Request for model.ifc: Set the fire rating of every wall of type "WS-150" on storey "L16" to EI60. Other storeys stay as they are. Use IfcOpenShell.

First a look at what the model holds.

```python
import ifcopenshell
import ifcopenshell.util.element

model = ifcopenshell.open("model.ifc")
print(model.schema)
storey = next(s for s in model.by_type("IfcBuildingStorey") if s.Name == "L16")
walls = [e for e in ifcopenshell.util.element.get_decomposition(storey) if e.is_a("IfcWall")]
seen = {}
for e in walls:
    element_type = ifcopenshell.util.element.get_type(e)
    key = (element_type.Name if element_type != e and element_type else None, ifcopenshell.util.element.get_pset(e, "Pset_WallCommon", "FireRating"))
    seen[key] = seen.get(key, 0) + 1
for (name, value), count in sorted(seen.items(), key=str):
    print(count, "x", name, "|", value)
```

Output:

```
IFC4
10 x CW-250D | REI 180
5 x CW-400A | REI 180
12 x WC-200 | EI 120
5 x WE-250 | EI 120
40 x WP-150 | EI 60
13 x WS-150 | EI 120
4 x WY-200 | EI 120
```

```python
import ifcopenshell
import ifcopenshell.api.pset
import ifcopenshell.util.element

model = ifcopenshell.open("model.ifc")

storey = next(s for s in model.by_type("IfcBuildingStorey") if s.Name == "L16")
walls = [e for e in ifcopenshell.util.element.get_decomposition(storey) if e.is_a("IfcWall")]

count = 0
for e in walls:
    element_type = ifcopenshell.util.element.get_type(e)
    if element_type in (None, e) or element_type.Name != "WS-150":
        continue
    found = ifcopenshell.util.element.get_pset(e, "Pset_WallCommon", should_inherit=False)
    if found:
        pset = model.by_id(found["id"])
        if len(ifcopenshell.util.element.get_elements_by_pset(pset)) > 1:
            pset = ifcopenshell.api.pset.unshare_pset(model, products=[e], pset=pset)[0]
    else:
        pset = ifcopenshell.api.pset.add_pset(model, product=e, name="Pset_WallCommon")
    ifcopenshell.api.pset.edit_pset(model, pset=pset, properties={"FireRating": "EI60"})
    count += 1

print(count, "walls updated")

model.write("model-out.ifc")
```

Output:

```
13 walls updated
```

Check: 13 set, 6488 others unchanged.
